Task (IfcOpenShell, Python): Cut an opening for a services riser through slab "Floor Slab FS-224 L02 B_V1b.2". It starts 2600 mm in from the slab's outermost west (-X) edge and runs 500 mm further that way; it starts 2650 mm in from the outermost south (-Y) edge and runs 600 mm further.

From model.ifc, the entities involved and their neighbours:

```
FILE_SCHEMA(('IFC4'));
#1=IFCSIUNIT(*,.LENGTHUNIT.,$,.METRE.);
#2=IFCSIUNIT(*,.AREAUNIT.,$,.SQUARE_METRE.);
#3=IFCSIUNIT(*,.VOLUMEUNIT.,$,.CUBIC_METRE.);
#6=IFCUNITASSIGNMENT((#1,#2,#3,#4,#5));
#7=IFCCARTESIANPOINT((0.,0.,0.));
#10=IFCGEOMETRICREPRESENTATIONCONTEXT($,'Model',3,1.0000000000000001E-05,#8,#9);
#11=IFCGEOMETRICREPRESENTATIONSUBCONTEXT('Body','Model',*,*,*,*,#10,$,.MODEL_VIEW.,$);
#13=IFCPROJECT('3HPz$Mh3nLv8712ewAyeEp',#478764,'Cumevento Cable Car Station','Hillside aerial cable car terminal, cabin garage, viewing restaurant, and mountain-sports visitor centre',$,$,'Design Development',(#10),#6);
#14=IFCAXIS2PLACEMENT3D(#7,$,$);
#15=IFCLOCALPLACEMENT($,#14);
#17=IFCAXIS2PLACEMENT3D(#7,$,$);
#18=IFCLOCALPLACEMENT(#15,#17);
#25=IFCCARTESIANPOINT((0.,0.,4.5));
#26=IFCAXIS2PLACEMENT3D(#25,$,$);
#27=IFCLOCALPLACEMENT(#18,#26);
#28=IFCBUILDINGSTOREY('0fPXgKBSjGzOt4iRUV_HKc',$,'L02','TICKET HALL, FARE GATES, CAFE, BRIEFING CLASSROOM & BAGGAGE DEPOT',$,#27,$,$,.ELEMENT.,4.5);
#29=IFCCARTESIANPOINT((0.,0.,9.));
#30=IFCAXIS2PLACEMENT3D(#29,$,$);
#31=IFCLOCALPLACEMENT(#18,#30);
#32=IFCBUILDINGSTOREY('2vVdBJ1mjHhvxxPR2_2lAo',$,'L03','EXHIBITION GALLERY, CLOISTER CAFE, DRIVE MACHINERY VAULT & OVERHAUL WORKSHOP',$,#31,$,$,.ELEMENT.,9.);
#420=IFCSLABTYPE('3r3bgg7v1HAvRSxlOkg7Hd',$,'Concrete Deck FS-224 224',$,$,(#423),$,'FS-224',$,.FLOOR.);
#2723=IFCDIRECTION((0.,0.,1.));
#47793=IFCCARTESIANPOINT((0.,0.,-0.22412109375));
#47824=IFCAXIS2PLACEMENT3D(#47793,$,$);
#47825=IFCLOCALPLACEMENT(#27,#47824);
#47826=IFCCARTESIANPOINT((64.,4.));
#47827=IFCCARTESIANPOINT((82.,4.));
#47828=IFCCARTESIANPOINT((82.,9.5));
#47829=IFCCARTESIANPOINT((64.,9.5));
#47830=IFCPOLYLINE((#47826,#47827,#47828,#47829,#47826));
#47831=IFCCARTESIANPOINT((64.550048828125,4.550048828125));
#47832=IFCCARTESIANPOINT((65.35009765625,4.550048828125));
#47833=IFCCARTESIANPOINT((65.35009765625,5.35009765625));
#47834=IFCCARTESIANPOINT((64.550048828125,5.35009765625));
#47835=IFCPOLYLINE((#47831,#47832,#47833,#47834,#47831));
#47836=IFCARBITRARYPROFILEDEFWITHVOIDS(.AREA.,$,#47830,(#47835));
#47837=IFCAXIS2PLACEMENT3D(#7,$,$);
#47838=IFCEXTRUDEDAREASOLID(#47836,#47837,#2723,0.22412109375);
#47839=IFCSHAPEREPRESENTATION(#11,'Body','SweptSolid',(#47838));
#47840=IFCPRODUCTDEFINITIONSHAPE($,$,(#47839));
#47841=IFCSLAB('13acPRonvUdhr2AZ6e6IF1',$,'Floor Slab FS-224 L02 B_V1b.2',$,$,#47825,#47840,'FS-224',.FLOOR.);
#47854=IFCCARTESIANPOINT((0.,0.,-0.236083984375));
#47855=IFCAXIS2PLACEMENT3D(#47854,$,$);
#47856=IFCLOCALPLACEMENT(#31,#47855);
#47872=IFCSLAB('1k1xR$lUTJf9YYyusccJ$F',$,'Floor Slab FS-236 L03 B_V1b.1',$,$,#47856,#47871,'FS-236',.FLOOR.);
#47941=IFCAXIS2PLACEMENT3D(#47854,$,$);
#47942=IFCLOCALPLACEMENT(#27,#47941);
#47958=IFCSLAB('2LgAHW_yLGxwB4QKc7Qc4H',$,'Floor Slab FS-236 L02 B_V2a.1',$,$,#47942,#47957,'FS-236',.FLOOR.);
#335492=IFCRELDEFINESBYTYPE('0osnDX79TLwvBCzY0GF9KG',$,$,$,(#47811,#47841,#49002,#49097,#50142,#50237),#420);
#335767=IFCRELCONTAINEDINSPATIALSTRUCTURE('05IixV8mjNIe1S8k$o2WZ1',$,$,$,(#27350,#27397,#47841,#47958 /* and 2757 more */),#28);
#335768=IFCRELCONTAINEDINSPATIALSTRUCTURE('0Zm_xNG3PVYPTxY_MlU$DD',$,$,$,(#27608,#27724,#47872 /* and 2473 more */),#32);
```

```python
import numpy as np
import ifcopenshell
import ifcopenshell.api.feature
import ifcopenshell.api.geometry
import ifcopenshell.api.root
import ifcopenshell.geom
import ifcopenshell.util.placement
import ifcopenshell.util.representation
import ifcopenshell.util.shape
import ifcopenshell.util.unit

model = ifcopenshell.open("model.ifc")
unit_scale = ifcopenshell.util.unit.calculate_unit_scale(model)
settings = ifcopenshell.geom.settings()


def volume(element):
    """Net volume in cubic metres, openings subtracted."""
    shape = ifcopenshell.geom.create_shape(settings, element)
    return ifcopenshell.util.shape.get_volume(shape.geometry)


slab = model.by_guid("13acPRonvUdhr2AZ6e6IF1")
before = volume(slab)

# Extent in the slab's own axes, in metres. The edges named are its -X and -Y sides.
slab_shape = ifcopenshell.geom.create_shape(settings, slab)
vertices = ifcopenshell.util.shape.get_vertices(slab_shape.geometry)
x_min, y_min, bottom = vertices.min(axis=0)
top = vertices[:, 2].max()

opening = ifcopenshell.api.root.create_entity(model, ifc_class="IfcOpeningElement", name="Services riser opening", predefined_type="OPENING")
context = ifcopenshell.util.representation.get_context(model, "Model", "Body", "MODEL_VIEW")
width, depth = 0.5, 0.6
outline = [(0.0, 0.0), (width, 0.0), (width, depth), (0.0, depth), (0.0, 0.0)]
# Overshoot both faces by 50 mm so the cut is clean.
shape = ifcopenshell.api.geometry.add_slab_representation(
    model, context=context, depth=top - bottom + 0.1, polyline=outline
)
ifcopenshell.api.geometry.assign_representation(model, product=opening, representation=shape)

matrix = ifcopenshell.util.placement.get_local_placement(slab.ObjectPlacement)
matrix[:, 3] = matrix @ np.append(np.array([x_min + 2.6, y_min + 2.65, bottom - 0.05]) / unit_scale, 1.0)
ifcopenshell.api.geometry.edit_object_placement(model, product=opening, matrix=matrix, is_si=False)
ifcopenshell.api.feature.add_feature(model, feature=opening, element=slab)

after = volume(slab)

print(f"slab volume {before:.3f} -> {after:.3f} m3")

model.write("model_v2.ifc")
```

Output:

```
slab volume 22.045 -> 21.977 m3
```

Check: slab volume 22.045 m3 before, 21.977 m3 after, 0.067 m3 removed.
